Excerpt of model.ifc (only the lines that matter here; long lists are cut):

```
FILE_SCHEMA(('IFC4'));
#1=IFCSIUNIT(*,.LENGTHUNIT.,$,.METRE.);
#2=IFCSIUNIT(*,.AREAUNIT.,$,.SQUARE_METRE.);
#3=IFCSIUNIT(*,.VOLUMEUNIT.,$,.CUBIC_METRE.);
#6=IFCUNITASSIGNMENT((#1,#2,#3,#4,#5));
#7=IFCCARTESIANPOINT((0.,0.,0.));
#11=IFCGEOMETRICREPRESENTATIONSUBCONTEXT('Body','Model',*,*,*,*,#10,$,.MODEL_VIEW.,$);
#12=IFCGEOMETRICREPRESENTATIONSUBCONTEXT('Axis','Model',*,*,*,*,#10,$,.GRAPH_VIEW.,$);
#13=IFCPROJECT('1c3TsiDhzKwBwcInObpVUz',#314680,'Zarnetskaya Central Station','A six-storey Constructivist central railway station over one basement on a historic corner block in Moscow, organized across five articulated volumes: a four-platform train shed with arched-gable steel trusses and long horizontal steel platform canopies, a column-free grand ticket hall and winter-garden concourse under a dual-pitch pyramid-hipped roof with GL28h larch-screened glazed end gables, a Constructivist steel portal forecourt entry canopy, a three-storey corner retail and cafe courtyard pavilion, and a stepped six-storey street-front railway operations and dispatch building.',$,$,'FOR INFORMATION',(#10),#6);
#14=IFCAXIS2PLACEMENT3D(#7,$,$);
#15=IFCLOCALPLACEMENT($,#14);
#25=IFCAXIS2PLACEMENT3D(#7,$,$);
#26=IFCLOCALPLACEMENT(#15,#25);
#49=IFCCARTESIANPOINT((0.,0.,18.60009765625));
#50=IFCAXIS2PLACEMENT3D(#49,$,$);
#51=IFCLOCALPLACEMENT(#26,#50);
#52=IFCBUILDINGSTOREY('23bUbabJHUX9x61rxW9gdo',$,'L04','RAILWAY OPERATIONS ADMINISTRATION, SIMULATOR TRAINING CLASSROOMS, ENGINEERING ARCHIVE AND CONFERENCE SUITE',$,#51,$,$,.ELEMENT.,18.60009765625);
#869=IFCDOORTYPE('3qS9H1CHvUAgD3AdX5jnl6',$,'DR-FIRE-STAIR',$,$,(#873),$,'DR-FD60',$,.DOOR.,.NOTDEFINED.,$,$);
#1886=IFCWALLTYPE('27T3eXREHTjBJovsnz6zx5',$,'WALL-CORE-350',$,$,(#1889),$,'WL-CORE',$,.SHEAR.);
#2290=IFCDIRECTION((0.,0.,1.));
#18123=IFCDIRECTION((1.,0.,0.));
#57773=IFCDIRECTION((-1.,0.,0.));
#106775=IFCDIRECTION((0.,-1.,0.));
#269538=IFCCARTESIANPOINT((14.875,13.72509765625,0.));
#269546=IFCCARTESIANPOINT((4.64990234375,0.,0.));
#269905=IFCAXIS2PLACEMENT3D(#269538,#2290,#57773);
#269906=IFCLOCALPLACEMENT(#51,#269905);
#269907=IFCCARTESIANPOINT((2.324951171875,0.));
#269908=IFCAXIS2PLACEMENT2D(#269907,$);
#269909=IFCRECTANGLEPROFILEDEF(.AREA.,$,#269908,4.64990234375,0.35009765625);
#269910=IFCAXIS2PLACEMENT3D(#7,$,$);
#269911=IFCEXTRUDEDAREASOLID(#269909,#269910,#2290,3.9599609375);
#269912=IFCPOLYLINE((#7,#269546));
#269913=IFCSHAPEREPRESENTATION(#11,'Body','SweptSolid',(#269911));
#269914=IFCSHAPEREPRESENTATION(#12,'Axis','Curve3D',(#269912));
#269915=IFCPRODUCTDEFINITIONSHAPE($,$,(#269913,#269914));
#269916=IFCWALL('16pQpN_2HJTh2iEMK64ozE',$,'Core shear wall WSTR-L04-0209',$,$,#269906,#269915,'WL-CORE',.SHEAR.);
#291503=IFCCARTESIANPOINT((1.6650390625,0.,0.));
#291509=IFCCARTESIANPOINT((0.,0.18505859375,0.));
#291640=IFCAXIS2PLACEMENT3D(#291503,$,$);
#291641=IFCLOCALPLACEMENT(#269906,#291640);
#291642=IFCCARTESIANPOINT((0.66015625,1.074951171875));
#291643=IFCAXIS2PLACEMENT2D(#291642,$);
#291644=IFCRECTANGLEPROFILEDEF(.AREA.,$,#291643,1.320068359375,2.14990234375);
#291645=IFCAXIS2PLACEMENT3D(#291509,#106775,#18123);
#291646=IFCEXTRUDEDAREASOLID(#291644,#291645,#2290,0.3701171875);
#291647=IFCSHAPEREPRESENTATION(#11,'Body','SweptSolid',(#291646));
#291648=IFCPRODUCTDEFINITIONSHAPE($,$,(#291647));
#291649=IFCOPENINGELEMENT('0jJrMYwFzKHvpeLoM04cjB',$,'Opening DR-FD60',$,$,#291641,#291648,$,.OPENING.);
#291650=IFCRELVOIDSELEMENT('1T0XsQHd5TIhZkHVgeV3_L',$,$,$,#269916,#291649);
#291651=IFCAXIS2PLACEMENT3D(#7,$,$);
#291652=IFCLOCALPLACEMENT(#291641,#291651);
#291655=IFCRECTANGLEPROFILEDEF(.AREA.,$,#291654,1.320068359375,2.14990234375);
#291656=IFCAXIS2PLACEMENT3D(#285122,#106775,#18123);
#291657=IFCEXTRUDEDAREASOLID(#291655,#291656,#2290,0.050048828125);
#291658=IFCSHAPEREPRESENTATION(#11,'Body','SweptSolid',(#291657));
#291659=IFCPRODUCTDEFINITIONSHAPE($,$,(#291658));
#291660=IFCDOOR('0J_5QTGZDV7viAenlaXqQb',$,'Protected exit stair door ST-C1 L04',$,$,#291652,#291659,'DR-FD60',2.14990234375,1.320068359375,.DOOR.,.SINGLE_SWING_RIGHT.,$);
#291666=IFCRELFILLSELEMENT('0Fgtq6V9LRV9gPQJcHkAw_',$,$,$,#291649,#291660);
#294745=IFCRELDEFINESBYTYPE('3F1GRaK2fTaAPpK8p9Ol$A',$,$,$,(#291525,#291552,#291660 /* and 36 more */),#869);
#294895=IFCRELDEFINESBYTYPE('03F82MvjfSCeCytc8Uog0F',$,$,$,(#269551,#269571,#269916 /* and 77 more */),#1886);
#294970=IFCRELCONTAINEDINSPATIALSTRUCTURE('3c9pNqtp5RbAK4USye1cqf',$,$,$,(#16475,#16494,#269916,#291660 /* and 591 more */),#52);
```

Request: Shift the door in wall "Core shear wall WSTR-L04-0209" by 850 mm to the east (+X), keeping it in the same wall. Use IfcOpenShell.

```python
import ifcopenshell
import ifcopenshell.api.geometry
import ifcopenshell.util.placement

model = ifcopenshell.open("model.ifc")

door = model.by_id(291660)
opening = door.FillsVoids[0].RelatingOpeningElement
wall = opening.VoidsElements[0].RelatingBuildingElement

wall_matrix = ifcopenshell.util.placement.get_local_placement(wall.ObjectPlacement)
shift = wall_matrix[:3, 0] * -0.85
before = ifcopenshell.util.placement.get_local_placement(door.ObjectPlacement)[:3, 3].copy()

# The door is placed relative to its opening, so it follows when the opening moves.
matrix = ifcopenshell.util.placement.get_local_placement(opening.ObjectPlacement)
matrix[:3, 3] += shift
ifcopenshell.api.geometry.edit_object_placement(
    model, product=opening, matrix=matrix, is_si=False, should_transform_children=True
)

after = ifcopenshell.util.placement.get_local_placement(door.ObjectPlacement)[:3, 3]
print("door moved by", (after - before).round(3) + 0.0)

model.write("model_edited.ifc")
```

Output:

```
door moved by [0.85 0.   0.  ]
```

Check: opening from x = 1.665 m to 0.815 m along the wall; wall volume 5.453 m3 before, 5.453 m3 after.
